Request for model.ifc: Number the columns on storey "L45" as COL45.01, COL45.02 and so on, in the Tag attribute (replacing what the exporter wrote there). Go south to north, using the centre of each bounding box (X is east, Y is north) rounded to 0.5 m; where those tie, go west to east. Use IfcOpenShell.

First a look at what the model holds.

```python
import ifcopenshell
import ifcopenshell.util.element
import ifcopenshell.util.placement

model = ifcopenshell.open("model.ifc")
print(model.schema)
storey = next(s for s in model.by_type("IfcBuildingStorey") if s.Name == "L45")
columns = [e for e in ifcopenshell.util.element.get_decomposition(storey) if e.is_a("IfcColumn")]
for e in sorted(columns, key=lambda e: e.id()):
    origin = ifcopenshell.util.placement.get_local_placement(e.ObjectPlacement)[:3, 3]
    print(e.id(), e.Tag, e.Name, origin.round(2) + 0.0, sep=" | ")
```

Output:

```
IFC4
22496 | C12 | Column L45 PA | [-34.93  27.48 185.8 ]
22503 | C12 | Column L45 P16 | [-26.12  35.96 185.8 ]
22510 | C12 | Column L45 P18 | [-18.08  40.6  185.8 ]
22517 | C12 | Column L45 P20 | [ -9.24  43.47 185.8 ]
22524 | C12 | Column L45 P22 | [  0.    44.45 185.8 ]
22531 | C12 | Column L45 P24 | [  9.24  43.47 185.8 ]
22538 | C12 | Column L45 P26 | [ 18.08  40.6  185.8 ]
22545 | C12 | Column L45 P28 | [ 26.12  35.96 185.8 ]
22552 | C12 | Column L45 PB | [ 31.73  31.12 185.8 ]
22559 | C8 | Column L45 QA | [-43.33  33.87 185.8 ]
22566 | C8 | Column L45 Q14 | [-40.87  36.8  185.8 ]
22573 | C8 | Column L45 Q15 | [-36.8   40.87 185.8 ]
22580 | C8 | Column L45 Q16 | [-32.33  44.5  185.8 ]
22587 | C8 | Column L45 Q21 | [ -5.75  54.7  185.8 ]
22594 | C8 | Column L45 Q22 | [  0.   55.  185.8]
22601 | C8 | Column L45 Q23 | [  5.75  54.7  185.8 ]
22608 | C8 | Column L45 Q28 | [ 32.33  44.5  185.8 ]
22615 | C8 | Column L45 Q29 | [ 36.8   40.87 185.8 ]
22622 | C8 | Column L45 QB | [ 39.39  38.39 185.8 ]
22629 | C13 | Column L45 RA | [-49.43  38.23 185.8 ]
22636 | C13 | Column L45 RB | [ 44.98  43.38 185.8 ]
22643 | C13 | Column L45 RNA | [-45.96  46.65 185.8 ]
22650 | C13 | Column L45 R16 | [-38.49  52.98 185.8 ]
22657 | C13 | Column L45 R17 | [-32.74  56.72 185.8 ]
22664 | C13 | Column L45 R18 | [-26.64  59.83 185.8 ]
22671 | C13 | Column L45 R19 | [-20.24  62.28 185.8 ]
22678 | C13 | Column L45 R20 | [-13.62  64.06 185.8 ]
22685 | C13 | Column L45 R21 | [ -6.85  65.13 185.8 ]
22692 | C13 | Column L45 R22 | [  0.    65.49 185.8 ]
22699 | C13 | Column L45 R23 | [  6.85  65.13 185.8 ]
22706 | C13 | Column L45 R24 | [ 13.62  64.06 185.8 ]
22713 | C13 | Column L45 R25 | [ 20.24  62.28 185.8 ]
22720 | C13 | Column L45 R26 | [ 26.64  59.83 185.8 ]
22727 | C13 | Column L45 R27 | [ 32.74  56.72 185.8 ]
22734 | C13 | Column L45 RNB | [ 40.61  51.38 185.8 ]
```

```python
import ifcopenshell
import ifcopenshell.geom
import ifcopenshell.util.element
import ifcopenshell.util.shape

model = ifcopenshell.open("model.ifc")
settings = ifcopenshell.geom.settings()
settings.set("use-world-coords", True)


def centre(element):
    shape = ifcopenshell.geom.create_shape(settings, element)
    return ifcopenshell.util.shape.get_bbox_centroid(shape.geometry)


storey = next(s for s in model.by_type("IfcBuildingStorey") if s.Name == "L45")
columns = [e for e in ifcopenshell.util.element.get_decomposition(storey) if e.is_a("IfcColumn")]

# Insertion points can sit at a corner or the storey origin, so sort by the geometry (in metres).
centres = {e: centre(e) for e in columns}
columns.sort(key=lambda e: (round(centres[e][1] / 0.5), centres[e][0]))

for i, e in enumerate(columns, start=1):
    number = f"COL45.{i:02d}"
    e.Tag = number
    print(e.id(), number)

model.write("model_updated.ifc")
```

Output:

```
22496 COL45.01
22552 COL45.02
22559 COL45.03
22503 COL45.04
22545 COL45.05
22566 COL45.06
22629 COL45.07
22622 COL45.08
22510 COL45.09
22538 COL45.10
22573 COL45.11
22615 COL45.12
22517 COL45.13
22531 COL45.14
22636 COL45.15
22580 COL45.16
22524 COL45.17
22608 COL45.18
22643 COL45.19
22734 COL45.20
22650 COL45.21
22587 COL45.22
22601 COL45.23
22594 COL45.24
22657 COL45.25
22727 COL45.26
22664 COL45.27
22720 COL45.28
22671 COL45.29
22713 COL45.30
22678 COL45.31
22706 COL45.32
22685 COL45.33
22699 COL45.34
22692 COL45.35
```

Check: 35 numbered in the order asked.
